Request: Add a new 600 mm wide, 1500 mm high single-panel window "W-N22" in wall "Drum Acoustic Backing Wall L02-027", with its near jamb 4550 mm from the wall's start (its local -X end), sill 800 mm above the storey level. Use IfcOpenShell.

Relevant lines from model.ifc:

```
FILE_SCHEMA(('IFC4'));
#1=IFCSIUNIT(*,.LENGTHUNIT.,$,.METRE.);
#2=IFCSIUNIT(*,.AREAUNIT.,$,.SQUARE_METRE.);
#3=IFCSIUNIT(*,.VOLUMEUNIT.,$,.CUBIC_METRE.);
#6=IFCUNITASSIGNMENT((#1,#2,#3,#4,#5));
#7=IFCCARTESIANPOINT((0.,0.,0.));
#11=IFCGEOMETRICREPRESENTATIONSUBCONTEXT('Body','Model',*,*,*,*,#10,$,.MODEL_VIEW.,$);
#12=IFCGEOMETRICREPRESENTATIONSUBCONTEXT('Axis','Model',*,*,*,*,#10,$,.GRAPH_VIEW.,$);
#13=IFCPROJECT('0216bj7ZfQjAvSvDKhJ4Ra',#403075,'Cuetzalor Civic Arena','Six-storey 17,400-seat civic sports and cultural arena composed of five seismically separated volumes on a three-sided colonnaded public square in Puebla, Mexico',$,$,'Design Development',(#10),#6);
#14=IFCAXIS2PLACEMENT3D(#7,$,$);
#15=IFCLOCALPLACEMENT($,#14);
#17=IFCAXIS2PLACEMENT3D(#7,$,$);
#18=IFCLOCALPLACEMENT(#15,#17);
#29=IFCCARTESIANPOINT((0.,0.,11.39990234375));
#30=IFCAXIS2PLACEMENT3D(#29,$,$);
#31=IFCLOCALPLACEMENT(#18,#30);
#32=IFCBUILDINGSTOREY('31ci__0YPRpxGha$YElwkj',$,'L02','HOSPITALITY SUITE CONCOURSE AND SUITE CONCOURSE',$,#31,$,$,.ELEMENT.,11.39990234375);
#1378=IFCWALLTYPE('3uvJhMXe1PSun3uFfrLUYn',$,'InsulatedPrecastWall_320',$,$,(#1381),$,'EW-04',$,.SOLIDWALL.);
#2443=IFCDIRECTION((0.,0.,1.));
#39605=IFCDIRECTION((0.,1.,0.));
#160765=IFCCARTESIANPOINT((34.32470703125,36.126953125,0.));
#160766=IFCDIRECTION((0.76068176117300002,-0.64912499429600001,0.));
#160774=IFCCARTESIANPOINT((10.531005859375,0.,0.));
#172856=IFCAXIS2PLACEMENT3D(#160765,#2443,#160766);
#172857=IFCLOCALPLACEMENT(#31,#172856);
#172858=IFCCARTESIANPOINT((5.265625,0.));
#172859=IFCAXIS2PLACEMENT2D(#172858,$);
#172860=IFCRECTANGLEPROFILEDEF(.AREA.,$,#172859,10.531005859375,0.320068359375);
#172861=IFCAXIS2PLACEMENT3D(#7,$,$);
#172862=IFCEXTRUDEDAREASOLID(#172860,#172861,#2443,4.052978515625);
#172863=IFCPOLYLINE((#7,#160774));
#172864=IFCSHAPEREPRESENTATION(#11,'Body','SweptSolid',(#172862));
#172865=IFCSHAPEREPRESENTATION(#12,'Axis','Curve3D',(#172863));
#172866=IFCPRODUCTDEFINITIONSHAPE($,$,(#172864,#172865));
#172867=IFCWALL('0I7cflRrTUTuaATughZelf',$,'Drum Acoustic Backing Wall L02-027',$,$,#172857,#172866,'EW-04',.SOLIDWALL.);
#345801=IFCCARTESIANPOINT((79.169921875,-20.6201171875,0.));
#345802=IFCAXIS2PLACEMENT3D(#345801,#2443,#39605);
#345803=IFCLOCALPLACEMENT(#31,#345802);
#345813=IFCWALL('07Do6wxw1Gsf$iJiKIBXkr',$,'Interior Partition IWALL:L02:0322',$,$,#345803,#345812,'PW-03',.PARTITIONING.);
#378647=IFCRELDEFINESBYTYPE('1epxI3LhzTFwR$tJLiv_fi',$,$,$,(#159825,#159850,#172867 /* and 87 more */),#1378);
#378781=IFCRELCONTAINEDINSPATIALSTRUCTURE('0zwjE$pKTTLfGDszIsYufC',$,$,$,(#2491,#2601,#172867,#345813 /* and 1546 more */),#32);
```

```python
import numpy as np
import ifcopenshell
import ifcopenshell.api.feature
import ifcopenshell.api.geometry
import ifcopenshell.api.root
import ifcopenshell.api.spatial
import ifcopenshell.geom
import ifcopenshell.util.element
import ifcopenshell.util.placement
import ifcopenshell.util.representation
import ifcopenshell.util.shape
import ifcopenshell.util.unit

model = ifcopenshell.open("model.ifc")
unit_scale = ifcopenshell.util.unit.calculate_unit_scale(model)
settings = ifcopenshell.geom.settings()


def volume(element):
    """Net volume in cubic metres, openings subtracted."""
    shape = ifcopenshell.geom.create_shape(settings, element)
    return ifcopenshell.util.shape.get_volume(shape.geometry)


wall = model.by_guid("0I7cflRrTUTuaATughZelf")
storey = ifcopenshell.util.element.get_container(wall, ifc_class="IfcBuildingStorey")
context = ifcopenshell.util.representation.get_context(model, "Model", "Body", "MODEL_VIEW")
before = volume(wall)

width, height, from_end, sill = 0.6, 1.5, 4.55, 0.8  # metres

# The wall runs along its own X axis, and the end named is its -X end.
wall_shape = ifcopenshell.geom.create_shape(settings, wall)
x, y, z = ifcopenshell.util.shape.get_vertices(wall_shape.geometry).T
start = x.min() + from_end
face, thickness = float(y.min()), float(y.max() - y.min())
wall_matrix = ifcopenshell.util.placement.get_local_placement(wall.ObjectPlacement)
level = ifcopenshell.util.placement.get_local_placement(storey.ObjectPlacement)[2, 3]


def in_wall(x, y):
    """Placement at x, y metres in the wall's axes, at sill height."""
    matrix = wall_matrix.copy()
    matrix[:, 3] = wall_matrix @ np.array([x / unit_scale, y / unit_scale, 0.0, 1.0])
    matrix[2, 3] = level + sill / unit_scale
    return matrix


# Opening: a box that overshoots both wall faces by 50 mm.
opening = ifcopenshell.api.root.create_entity(model, ifc_class="IfcOpeningElement", predefined_type="OPENING")
box = ifcopenshell.api.geometry.add_wall_representation(
    model, context=context, length=width, height=height, thickness=thickness + 0.1
)
ifcopenshell.api.geometry.assign_representation(model, product=opening, representation=box)
ifcopenshell.api.geometry.edit_object_placement(model, product=opening, matrix=in_wall(start, face - 0.05), is_si=False)
ifcopenshell.api.feature.add_feature(model, feature=opening, element=wall)

window = ifcopenshell.api.root.create_entity(model, ifc_class="IfcWindow", name="W-N22", predefined_type="WINDOW")
window.OverallWidth, window.OverallHeight = width / unit_scale, height / unit_scale
window.PartitioningType = "SINGLE_PANEL"
body = ifcopenshell.api.geometry.add_window_representation(
    model,
    context=context,
    overall_width=window.OverallWidth,
    overall_height=window.OverallHeight,
    partition_type="SINGLE_PANEL",
)
ifcopenshell.api.geometry.assign_representation(model, product=window, representation=body)
ifcopenshell.api.spatial.assign_container(model, products=[window], relating_structure=storey)
ifcopenshell.api.feature.add_filling(model, opening=opening, element=window)

# Centre the window in the wall's thickness.
ifcopenshell.api.geometry.edit_object_placement(model, product=window, matrix=in_wall(start, face), is_si=False)
window_shape = ifcopenshell.geom.create_shape(settings, window)
depth = ifcopenshell.util.shape.get_vertices(window_shape.geometry)[:, 1]
offset = face + thickness / 2 - (depth.min() + depth.max()) / 2
ifcopenshell.api.geometry.edit_object_placement(model, product=window, matrix=in_wall(start, offset), is_si=False)

after = volume(wall)

print(f"wall volume {before:.3f} -> {after:.3f} m3")

model.write("model_rev.ifc")
```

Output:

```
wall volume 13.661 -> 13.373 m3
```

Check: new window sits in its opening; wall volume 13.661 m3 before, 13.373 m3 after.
